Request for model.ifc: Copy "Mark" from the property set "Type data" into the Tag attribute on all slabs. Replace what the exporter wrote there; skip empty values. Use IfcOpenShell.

First a look at what the model holds.

```python
import ifcopenshell
import ifcopenshell.util.element

model = ifcopenshell.open("model.ifc")
print(model.schema)
slabs = model.by_type("IfcSlab")
print(len(slabs), "slabs")
for e in slabs[:8]:
    source = ifcopenshell.util.element.get_pset(e, "Type data", "Mark")
    target = e.Tag
    print(e.id(), repr(source), repr(target), sep=" | ")
```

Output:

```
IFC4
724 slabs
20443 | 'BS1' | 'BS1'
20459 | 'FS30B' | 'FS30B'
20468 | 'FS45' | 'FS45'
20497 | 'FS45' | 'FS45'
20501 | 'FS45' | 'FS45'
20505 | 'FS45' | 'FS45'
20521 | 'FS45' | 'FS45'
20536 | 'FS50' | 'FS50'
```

```python
import ifcopenshell
import ifcopenshell.util.element

model = ifcopenshell.open("model.ifc")

count = 0
for e in model.by_type("IfcSlab"):
    value = ifcopenshell.util.element.get_pset(e, "Type data", "Mark")
    current = e.Tag
    if not value or not value.strip() or current == value:
        continue
    e.Tag = value
    count += 1

print(count, "slabs updated")

model.write("model_updated.ifc")
```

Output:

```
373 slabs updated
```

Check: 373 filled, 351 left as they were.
